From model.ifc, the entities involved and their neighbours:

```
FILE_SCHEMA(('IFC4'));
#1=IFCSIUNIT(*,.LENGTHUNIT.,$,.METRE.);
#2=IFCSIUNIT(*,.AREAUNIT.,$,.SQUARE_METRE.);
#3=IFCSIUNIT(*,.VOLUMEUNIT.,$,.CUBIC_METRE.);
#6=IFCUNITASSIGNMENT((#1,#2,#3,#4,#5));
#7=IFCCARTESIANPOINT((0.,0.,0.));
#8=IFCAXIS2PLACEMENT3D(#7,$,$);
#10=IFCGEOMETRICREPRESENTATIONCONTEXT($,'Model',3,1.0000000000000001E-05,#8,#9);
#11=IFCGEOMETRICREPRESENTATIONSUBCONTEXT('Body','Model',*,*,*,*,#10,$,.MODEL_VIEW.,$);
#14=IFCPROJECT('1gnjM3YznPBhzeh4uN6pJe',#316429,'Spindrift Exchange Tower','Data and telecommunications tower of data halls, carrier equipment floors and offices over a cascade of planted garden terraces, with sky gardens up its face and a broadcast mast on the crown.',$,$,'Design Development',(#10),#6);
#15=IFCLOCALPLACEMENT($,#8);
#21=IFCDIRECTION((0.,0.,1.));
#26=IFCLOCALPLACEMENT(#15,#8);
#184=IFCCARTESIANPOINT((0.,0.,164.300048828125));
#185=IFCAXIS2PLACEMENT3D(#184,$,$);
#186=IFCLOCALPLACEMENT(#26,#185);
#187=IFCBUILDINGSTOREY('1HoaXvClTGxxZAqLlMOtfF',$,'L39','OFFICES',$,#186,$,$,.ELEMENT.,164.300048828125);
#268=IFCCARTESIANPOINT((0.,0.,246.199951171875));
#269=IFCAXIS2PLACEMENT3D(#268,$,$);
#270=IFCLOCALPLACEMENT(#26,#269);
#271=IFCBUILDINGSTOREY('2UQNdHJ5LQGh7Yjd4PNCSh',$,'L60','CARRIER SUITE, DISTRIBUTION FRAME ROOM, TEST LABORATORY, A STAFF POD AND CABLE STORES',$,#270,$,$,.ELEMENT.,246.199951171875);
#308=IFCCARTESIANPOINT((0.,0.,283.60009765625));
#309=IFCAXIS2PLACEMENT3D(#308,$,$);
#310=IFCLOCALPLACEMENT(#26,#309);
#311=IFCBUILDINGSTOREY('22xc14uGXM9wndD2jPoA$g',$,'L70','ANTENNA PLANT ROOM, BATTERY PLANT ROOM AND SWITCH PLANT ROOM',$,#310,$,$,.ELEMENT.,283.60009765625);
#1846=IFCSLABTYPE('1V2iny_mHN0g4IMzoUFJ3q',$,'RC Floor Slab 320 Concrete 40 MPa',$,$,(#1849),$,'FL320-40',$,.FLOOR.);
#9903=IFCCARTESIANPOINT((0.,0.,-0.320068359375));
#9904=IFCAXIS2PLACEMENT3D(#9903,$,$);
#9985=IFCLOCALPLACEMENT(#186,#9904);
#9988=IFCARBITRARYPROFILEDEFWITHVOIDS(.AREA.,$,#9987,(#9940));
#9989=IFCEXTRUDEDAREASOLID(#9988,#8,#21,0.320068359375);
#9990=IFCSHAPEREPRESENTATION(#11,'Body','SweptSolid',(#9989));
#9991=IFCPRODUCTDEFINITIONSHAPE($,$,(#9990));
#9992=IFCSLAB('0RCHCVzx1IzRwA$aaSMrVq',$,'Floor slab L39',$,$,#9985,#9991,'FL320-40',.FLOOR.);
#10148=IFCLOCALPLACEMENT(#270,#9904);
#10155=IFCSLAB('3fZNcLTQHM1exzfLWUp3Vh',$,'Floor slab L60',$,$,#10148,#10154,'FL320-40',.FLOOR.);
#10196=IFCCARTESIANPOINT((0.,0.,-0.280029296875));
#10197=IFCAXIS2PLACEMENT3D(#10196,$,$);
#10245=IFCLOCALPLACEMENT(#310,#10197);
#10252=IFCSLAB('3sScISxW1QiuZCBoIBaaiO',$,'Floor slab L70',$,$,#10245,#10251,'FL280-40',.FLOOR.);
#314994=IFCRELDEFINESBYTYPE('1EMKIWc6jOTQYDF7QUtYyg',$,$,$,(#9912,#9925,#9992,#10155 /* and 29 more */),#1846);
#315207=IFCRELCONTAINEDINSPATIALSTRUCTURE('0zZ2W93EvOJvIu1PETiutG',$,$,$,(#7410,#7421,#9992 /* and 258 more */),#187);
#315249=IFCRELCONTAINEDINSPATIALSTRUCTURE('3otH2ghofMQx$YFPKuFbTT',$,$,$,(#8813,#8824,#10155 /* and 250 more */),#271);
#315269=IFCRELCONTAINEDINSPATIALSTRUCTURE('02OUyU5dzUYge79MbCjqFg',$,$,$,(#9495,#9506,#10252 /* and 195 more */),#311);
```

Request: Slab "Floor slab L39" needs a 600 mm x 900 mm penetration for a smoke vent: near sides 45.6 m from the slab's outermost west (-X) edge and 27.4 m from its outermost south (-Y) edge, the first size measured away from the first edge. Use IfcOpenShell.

```python
import numpy as np
import ifcopenshell
import ifcopenshell.api.feature
import ifcopenshell.api.geometry
import ifcopenshell.api.root
import ifcopenshell.geom
import ifcopenshell.util.placement
import ifcopenshell.util.representation
import ifcopenshell.util.shape
import ifcopenshell.util.unit

model = ifcopenshell.open("model.ifc")
unit_scale = ifcopenshell.util.unit.calculate_unit_scale(model)
settings = ifcopenshell.geom.settings()


def volume(element):
    """Net volume in cubic metres, openings subtracted."""
    shape = ifcopenshell.geom.create_shape(settings, element)
    return ifcopenshell.util.shape.get_volume(shape.geometry)


slab = model.by_guid("0RCHCVzx1IzRwA$aaSMrVq")
before = volume(slab)

# Extent in the slab's own axes, in metres. The edges named are its -X and -Y sides.
slab_shape = ifcopenshell.geom.create_shape(settings, slab)
vertices = ifcopenshell.util.shape.get_vertices(slab_shape.geometry)
x_min, y_min, bottom = vertices.min(axis=0)
top = vertices[:, 2].max()

opening = ifcopenshell.api.root.create_entity(model, ifc_class="IfcOpeningElement", name="Smoke vent opening", predefined_type="OPENING")
context = ifcopenshell.util.representation.get_context(model, "Model", "Body", "MODEL_VIEW")
width, depth = 0.6, 0.9
outline = [(0.0, 0.0), (width, 0.0), (width, depth), (0.0, depth), (0.0, 0.0)]
# Overshoot both faces by 50 mm so the cut is clean.
shape = ifcopenshell.api.geometry.add_slab_representation(
    model, context=context, depth=top - bottom + 0.1, polyline=outline
)
ifcopenshell.api.geometry.assign_representation(model, product=opening, representation=shape)

matrix = ifcopenshell.util.placement.get_local_placement(slab.ObjectPlacement)
matrix[:, 3] = matrix @ np.append(np.array([x_min + 45.6, y_min + 27.4, bottom - 0.05]) / unit_scale, 1.0)
ifcopenshell.api.geometry.edit_object_placement(model, product=opening, matrix=matrix, is_si=False)
ifcopenshell.api.feature.add_feature(model, feature=opening, element=slab)

after = volume(slab)

print(f"slab volume {before:.3f} -> {after:.3f} m3")

model.write("model_updated.ifc")
```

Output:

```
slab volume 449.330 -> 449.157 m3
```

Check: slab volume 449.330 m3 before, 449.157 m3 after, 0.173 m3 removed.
